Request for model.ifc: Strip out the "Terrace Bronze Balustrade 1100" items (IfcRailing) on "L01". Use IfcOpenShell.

First a look at what the model holds.

```python
import ifcopenshell
import ifcopenshell.util.element

model = ifcopenshell.open("model.ifc")
print(model.schema)
storey = next(s for s in model.by_type("IfcBuildingStorey") if s.Name == "L01")
railings = [e for e in ifcopenshell.util.element.get_decomposition(storey) if e.is_a("IfcRailing")]
seen = {}
for e in railings:
    element_type = ifcopenshell.util.element.get_type(e)
    name = element_type.Name if element_type not in (None, e) else None
    seen[name] = seen.get(name, 0) + 1
for name, count in sorted(seen.items(), key=str):
    print(count, "x", name)
```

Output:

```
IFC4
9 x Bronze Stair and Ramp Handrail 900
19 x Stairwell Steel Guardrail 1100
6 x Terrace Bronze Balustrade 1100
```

```python
import ifcopenshell
import ifcopenshell.api.root
import ifcopenshell.util.element

model = ifcopenshell.open("model.ifc")

storey = next(s for s in model.by_type("IfcBuildingStorey") if s.Name == "L01")
railings = [e for e in ifcopenshell.util.element.get_decomposition(storey) if e.is_a("IfcRailing")]
targets = [e for e in railings if (t := ifcopenshell.util.element.get_type(e)) not in (None, e) and t.Name == "Terrace Bronze Balustrade 1100"]

for e in targets:
    ifcopenshell.api.root.remove_product(model, product=e)
print(len(targets), "removed")

model.write("model_edited.ifc")
```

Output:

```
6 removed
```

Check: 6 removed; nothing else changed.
